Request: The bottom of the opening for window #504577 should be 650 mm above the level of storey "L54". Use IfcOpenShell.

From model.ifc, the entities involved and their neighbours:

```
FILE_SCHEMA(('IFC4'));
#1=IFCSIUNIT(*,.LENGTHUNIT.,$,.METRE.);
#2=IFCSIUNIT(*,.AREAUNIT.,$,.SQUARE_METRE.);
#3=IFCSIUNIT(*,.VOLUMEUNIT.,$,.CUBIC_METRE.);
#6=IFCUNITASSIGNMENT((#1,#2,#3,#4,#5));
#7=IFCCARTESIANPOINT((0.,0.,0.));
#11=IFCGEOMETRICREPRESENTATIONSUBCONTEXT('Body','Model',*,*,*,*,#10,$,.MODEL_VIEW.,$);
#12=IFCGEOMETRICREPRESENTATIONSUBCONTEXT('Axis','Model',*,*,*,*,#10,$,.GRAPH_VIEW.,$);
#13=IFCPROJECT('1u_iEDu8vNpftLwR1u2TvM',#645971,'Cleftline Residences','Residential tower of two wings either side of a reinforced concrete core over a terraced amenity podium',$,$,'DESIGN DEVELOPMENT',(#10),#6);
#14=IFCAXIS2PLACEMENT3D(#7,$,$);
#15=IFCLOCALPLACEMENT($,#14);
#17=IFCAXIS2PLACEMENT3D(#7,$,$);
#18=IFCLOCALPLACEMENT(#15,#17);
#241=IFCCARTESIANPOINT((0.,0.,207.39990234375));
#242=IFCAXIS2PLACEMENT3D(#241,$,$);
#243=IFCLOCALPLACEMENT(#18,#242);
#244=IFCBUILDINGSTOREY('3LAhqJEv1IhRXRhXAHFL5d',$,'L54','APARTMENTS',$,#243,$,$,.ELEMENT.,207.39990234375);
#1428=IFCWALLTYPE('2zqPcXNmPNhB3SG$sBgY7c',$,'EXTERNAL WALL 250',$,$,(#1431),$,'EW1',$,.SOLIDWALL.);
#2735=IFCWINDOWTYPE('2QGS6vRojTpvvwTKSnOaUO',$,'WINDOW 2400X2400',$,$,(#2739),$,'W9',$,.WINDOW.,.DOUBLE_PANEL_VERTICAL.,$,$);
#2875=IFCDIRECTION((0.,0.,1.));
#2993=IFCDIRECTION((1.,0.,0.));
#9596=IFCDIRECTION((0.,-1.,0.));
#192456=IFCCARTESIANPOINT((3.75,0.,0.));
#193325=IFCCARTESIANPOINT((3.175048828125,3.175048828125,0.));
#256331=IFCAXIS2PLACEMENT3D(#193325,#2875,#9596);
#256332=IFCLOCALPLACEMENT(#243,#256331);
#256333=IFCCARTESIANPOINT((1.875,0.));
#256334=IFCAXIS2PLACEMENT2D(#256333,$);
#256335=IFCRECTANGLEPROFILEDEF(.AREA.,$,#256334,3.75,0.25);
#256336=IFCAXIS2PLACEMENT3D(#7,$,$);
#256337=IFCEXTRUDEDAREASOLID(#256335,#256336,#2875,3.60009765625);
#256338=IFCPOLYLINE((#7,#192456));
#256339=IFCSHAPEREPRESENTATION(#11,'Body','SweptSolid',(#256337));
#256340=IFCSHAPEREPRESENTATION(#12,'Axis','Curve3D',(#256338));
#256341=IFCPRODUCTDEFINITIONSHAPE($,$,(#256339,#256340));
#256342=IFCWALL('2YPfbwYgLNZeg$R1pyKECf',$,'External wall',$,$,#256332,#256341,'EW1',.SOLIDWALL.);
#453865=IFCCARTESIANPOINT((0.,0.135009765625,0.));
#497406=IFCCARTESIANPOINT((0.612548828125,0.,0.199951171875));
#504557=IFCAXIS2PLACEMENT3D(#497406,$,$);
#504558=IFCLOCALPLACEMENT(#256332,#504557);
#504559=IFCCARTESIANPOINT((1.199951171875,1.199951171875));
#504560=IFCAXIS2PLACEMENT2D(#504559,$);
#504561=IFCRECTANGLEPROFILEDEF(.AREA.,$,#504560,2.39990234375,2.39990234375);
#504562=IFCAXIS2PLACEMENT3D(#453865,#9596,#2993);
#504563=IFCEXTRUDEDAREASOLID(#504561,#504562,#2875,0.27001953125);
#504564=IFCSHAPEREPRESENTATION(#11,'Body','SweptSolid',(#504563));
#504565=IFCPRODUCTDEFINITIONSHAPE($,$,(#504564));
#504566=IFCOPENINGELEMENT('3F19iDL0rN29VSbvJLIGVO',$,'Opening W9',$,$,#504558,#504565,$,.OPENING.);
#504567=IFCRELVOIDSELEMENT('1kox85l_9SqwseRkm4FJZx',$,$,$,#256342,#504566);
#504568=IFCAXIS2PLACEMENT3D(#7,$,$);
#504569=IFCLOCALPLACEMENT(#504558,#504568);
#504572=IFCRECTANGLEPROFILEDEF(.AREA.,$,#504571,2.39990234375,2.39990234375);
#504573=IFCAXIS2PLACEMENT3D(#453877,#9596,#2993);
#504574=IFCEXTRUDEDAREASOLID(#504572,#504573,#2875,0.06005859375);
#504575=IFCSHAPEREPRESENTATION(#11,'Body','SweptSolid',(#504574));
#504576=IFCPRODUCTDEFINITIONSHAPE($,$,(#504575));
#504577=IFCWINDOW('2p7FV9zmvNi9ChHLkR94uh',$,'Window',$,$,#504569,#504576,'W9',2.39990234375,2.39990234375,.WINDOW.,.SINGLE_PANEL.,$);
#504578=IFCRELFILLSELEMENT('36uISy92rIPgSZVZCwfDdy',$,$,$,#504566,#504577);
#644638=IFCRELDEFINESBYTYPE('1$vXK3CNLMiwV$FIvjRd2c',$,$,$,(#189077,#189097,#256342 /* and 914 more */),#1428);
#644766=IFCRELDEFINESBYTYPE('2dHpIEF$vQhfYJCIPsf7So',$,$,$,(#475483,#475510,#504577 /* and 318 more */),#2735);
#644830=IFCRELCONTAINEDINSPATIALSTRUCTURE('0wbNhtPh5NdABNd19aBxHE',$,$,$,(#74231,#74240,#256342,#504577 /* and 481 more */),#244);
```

```python
import numpy as np
import ifcopenshell
import ifcopenshell.api.geometry
import ifcopenshell.geom
import ifcopenshell.util.element
import ifcopenshell.util.placement
import ifcopenshell.util.shape
import ifcopenshell.util.unit

model = ifcopenshell.open("model.ifc")
unit_scale = ifcopenshell.util.unit.calculate_unit_scale(model)

window = model.by_guid("2p7FV9zmvNi9ChHLkR94uh")
opening = window.FillsVoids[0].RelatingOpeningElement
storey = ifcopenshell.util.element.get_container(window, ifc_class="IfcBuildingStorey")
level = ifcopenshell.util.placement.get_local_placement(storey.ObjectPlacement)[2, 3]

# The opening's origin need not be at the sill, so measure its lowest point.
shape = ifcopenshell.geom.create_shape(ifcopenshell.geom.settings(), opening)
bottom = ifcopenshell.util.shape.get_shape_bottom_elevation(shape, shape.geometry) / unit_scale
dz = level + 0.65 / unit_scale - bottom

shift = np.array([0.0, 0.0, dz])
# The window is placed relative to its opening, so it follows when the opening moves.
matrix = ifcopenshell.util.placement.get_local_placement(opening.ObjectPlacement)
matrix[:3, 3] += shift
ifcopenshell.api.geometry.edit_object_placement(
    model, product=opening, matrix=matrix, is_si=False, should_transform_children=True
)

print(f"moved by {dz * unit_scale:+.3f} m")

model.write("model-out.ifc")
```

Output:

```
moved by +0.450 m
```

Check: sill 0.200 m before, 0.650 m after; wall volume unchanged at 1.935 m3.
